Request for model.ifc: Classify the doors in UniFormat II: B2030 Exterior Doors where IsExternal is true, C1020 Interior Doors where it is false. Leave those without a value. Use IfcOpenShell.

First a look at what the model holds.

```python
import ifcopenshell
import ifcopenshell.util.element

model = ifcopenshell.open("model.ifc")
print(model.schema)
print("classifications:", [c.Name for c in model.by_type("IfcClassification")])
values = [ifcopenshell.util.element.get_pset(e, "Pset_DoorCommon", "IsExternal") for e in model.by_type("IfcDoor")]
for value in (True, False, None):
    print("IsExternal", value, values.count(value))
```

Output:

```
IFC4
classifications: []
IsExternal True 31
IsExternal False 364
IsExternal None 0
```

```python
import ifcopenshell
import ifcopenshell.api.classification
import ifcopenshell.util.element

model = ifcopenshell.open("model.ifc")

system = ifcopenshell.api.classification.add_classification(model, classification="UniFormat II")

doors = model.by_type("IfcDoor")
external = {e: ifcopenshell.util.element.get_pset(e, "Pset_DoorCommon", "IsExternal") for e in doors}
for flag, code, name in ((True, "B2030", "Exterior Doors"), (False, "C1020", "Interior Doors")):
    products = [e for e in doors if external[e] is flag]
    ifcopenshell.api.classification.add_reference(
        model, products=products, classification=system, identification=code, name=name
    )
    print(code, len(products))

model.write("model-out.ifc")
```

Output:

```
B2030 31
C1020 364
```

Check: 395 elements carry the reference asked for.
